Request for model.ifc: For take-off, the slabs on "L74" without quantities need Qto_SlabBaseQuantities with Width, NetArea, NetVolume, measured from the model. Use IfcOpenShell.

First a look at what the model holds.

```python
import ifcopenshell
import ifcopenshell.util.element
import ifcopenshell.util.unit

model = ifcopenshell.open("model.ifc")
print(model.schema)
for unit_type in ("LENGTHUNIT", "AREAUNIT", "VOLUMEUNIT"):
    print(unit_type, ifcopenshell.util.unit.calculate_unit_scale(model, unit_type))
storey = next(s for s in model.by_type("IfcBuildingStorey") if s.Name == "L74")
slabs = [e for e in ifcopenshell.util.element.get_decomposition(storey) if e.is_a("IfcSlab")]
for e in sorted(slabs, key=lambda e: e.id()):
    print(e.id(), e.is_a(), e.Name, list(ifcopenshell.util.element.get_psets(e, qtos_only=True)), sep=" | ")
```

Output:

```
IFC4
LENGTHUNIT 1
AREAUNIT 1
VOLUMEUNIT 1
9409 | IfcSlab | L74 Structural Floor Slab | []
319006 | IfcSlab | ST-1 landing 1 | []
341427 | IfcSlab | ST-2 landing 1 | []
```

```python
import ifcopenshell
import ifcopenshell.api.pset
import ifcopenshell.geom
import ifcopenshell.util.element
import ifcopenshell.util.shape
import ifcopenshell.util.unit

model = ifcopenshell.open("model.ifc")
unit_scale = ifcopenshell.util.unit.calculate_unit_scale(model)
area_scale = ifcopenshell.util.unit.calculate_unit_scale(model, "AREAUNIT")
volume_scale = ifcopenshell.util.unit.calculate_unit_scale(model, "VOLUMEUNIT")
settings = ifcopenshell.geom.settings()

storey = next(s for s in model.by_type("IfcBuildingStorey") if s.Name == "L74")
slabs = [e for e in ifcopenshell.util.element.get_decomposition(storey) if e.is_a("IfcSlab")]

for e in sorted(slabs, key=lambda e: e.id()):
    if ifcopenshell.util.element.get_psets(e, qtos_only=True, should_inherit=False):
        continue
    # Geometry comes back in metres, in the element's own axes.
    shape = ifcopenshell.geom.create_shape(settings, e)
    values = {
        "Width": ifcopenshell.util.shape.get_z(shape.geometry) / unit_scale,
        "NetArea": ifcopenshell.util.shape.get_footprint_area(shape.geometry) / area_scale,
        "NetVolume": ifcopenshell.util.shape.get_volume(shape.geometry) / volume_scale,
    }
    qto = ifcopenshell.api.pset.add_qto(model, product=e, name="Qto_SlabBaseQuantities")
    ifcopenshell.api.pset.edit_qto(model, qto=qto, properties=values)
    print(e.id(), {k: round(v, 3) for k, v in values.items()})

model.write("model_edited.ifc")
```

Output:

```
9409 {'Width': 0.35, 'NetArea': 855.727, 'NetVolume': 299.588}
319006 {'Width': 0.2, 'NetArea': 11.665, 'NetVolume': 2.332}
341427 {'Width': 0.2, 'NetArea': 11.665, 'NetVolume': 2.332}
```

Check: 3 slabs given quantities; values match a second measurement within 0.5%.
